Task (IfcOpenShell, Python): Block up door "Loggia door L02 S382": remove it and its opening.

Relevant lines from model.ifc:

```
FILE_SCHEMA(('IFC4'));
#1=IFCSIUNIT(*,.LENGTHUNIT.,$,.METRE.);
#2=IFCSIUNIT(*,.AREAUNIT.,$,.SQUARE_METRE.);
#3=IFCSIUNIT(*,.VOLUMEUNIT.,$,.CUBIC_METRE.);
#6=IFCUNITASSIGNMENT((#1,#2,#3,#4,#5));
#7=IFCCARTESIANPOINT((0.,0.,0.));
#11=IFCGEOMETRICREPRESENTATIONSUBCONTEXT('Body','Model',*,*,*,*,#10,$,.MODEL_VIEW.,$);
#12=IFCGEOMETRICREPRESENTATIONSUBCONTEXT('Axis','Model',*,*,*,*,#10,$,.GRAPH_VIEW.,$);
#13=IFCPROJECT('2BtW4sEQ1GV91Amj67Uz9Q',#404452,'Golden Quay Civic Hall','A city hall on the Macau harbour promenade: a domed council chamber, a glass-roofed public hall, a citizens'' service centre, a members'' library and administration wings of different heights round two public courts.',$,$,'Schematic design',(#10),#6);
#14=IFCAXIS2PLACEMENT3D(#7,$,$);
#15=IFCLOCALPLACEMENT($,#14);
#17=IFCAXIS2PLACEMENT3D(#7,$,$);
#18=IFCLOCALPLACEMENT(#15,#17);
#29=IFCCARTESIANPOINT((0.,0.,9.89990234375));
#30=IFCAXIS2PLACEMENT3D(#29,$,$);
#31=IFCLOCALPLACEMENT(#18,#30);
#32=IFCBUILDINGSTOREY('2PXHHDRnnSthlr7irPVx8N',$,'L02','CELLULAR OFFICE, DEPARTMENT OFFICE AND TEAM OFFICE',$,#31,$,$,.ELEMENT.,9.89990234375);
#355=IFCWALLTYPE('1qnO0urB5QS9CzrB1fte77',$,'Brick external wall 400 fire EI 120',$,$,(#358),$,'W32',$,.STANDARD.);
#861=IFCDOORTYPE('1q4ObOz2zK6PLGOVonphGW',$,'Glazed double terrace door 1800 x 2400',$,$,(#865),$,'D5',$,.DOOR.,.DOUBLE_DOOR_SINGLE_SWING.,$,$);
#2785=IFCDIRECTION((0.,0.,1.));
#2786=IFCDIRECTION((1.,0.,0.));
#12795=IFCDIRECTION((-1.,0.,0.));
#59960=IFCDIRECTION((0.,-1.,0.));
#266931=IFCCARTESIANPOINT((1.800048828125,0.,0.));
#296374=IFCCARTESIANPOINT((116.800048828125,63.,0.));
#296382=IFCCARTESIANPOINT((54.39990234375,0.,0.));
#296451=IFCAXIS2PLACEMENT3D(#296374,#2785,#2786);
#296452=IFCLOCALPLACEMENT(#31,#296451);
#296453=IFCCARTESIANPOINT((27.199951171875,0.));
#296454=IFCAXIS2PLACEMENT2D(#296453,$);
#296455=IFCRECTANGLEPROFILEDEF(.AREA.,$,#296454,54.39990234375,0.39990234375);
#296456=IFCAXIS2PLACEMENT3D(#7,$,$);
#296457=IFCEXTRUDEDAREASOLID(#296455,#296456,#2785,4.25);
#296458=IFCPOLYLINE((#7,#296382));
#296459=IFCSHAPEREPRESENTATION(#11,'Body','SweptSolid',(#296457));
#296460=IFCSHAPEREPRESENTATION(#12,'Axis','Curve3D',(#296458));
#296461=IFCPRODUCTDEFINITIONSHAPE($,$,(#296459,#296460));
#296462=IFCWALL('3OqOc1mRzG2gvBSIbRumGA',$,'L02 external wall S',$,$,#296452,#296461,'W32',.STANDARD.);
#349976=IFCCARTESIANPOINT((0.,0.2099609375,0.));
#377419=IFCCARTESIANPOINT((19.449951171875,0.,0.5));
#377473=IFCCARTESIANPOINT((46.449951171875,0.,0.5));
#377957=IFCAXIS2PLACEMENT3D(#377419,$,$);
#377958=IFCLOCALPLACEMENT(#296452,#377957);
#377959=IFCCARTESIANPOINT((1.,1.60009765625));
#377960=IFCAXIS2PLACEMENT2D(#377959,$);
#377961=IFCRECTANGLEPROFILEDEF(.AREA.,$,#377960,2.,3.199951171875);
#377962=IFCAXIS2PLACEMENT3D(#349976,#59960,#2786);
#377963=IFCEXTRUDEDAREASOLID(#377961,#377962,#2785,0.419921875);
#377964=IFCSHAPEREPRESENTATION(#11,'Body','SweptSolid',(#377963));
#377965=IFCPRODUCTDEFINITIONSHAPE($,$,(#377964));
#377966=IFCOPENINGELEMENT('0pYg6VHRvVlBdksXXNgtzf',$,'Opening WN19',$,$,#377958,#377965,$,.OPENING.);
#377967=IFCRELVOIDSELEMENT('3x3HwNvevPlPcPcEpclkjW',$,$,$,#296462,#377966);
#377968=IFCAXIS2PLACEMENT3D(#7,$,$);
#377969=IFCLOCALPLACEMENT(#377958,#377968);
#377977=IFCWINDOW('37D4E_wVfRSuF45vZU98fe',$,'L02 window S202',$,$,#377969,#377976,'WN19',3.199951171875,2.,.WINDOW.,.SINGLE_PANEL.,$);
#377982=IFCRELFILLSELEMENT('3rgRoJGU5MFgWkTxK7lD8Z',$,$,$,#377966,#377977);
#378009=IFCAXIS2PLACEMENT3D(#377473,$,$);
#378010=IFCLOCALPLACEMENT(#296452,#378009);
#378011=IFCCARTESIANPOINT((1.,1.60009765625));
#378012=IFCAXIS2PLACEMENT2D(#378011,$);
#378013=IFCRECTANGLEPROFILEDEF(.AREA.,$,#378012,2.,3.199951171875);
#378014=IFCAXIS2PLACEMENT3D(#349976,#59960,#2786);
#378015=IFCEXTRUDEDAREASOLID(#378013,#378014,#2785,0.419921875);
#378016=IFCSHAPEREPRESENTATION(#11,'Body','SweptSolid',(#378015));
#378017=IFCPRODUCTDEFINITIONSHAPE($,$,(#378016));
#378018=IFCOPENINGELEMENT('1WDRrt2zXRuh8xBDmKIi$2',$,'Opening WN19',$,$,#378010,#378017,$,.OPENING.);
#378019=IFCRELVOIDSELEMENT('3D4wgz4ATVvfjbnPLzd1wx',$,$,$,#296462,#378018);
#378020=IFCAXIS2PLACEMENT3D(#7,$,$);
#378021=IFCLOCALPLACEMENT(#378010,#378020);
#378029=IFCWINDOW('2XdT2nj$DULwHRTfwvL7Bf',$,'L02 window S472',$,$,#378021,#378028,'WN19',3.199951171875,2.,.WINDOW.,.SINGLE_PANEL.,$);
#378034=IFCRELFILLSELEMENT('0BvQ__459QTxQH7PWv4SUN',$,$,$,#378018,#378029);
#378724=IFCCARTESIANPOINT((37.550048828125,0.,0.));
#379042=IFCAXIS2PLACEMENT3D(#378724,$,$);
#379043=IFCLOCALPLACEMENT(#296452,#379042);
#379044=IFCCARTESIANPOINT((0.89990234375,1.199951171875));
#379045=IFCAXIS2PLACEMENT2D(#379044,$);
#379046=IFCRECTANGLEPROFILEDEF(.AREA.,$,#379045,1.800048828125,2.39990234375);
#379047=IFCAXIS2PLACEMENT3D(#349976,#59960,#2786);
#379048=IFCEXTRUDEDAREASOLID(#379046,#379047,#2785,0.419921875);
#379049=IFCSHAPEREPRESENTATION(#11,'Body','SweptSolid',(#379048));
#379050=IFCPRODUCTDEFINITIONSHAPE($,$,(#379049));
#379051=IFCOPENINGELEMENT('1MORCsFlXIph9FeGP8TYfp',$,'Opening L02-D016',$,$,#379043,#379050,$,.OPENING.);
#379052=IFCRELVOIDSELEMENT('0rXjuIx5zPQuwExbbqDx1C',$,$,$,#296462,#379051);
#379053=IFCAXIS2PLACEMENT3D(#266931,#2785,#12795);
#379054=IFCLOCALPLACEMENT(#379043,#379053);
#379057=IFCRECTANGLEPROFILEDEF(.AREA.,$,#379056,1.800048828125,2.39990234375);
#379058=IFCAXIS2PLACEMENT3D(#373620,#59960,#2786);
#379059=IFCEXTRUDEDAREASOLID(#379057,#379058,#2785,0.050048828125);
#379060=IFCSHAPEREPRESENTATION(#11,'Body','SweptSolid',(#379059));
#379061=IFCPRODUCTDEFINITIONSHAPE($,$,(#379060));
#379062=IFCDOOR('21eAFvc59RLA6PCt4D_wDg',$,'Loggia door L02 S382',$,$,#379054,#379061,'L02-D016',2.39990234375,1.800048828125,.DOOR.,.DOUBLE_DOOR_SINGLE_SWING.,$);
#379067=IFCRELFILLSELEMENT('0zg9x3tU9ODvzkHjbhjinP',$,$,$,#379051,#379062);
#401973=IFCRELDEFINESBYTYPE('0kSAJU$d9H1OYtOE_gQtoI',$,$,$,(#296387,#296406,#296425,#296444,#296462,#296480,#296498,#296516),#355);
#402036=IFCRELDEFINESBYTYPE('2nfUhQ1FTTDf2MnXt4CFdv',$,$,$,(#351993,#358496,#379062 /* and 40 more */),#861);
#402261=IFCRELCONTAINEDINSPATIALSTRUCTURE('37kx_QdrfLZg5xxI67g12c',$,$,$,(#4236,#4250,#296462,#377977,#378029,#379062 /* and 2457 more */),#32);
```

```python
import ifcopenshell
import ifcopenshell.api.feature
import ifcopenshell.api.root
import ifcopenshell.geom
import ifcopenshell.util.shape

model = ifcopenshell.open("model.ifc")
settings = ifcopenshell.geom.settings()


def volume(element):
    """Net volume in cubic metres, openings subtracted."""
    shape = ifcopenshell.geom.create_shape(settings, element)
    return ifcopenshell.util.shape.get_volume(shape.geometry)


door = model.by_guid("21eAFvc59RLA6PCt4D_wDg")
opening = door.FillsVoids[0].RelatingOpeningElement
wall = opening.VoidsElements[0].RelatingBuildingElement
before = volume(wall)

ifcopenshell.api.root.remove_product(model, product=door)
ifcopenshell.api.feature.remove_feature(model, feature=opening)

after = volume(wall)

print(f"wall volume {before:.3f} -> {after:.3f} m3")

model.write("model_updated.ifc")
```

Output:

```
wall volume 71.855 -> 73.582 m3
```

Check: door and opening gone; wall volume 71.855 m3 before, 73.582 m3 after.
